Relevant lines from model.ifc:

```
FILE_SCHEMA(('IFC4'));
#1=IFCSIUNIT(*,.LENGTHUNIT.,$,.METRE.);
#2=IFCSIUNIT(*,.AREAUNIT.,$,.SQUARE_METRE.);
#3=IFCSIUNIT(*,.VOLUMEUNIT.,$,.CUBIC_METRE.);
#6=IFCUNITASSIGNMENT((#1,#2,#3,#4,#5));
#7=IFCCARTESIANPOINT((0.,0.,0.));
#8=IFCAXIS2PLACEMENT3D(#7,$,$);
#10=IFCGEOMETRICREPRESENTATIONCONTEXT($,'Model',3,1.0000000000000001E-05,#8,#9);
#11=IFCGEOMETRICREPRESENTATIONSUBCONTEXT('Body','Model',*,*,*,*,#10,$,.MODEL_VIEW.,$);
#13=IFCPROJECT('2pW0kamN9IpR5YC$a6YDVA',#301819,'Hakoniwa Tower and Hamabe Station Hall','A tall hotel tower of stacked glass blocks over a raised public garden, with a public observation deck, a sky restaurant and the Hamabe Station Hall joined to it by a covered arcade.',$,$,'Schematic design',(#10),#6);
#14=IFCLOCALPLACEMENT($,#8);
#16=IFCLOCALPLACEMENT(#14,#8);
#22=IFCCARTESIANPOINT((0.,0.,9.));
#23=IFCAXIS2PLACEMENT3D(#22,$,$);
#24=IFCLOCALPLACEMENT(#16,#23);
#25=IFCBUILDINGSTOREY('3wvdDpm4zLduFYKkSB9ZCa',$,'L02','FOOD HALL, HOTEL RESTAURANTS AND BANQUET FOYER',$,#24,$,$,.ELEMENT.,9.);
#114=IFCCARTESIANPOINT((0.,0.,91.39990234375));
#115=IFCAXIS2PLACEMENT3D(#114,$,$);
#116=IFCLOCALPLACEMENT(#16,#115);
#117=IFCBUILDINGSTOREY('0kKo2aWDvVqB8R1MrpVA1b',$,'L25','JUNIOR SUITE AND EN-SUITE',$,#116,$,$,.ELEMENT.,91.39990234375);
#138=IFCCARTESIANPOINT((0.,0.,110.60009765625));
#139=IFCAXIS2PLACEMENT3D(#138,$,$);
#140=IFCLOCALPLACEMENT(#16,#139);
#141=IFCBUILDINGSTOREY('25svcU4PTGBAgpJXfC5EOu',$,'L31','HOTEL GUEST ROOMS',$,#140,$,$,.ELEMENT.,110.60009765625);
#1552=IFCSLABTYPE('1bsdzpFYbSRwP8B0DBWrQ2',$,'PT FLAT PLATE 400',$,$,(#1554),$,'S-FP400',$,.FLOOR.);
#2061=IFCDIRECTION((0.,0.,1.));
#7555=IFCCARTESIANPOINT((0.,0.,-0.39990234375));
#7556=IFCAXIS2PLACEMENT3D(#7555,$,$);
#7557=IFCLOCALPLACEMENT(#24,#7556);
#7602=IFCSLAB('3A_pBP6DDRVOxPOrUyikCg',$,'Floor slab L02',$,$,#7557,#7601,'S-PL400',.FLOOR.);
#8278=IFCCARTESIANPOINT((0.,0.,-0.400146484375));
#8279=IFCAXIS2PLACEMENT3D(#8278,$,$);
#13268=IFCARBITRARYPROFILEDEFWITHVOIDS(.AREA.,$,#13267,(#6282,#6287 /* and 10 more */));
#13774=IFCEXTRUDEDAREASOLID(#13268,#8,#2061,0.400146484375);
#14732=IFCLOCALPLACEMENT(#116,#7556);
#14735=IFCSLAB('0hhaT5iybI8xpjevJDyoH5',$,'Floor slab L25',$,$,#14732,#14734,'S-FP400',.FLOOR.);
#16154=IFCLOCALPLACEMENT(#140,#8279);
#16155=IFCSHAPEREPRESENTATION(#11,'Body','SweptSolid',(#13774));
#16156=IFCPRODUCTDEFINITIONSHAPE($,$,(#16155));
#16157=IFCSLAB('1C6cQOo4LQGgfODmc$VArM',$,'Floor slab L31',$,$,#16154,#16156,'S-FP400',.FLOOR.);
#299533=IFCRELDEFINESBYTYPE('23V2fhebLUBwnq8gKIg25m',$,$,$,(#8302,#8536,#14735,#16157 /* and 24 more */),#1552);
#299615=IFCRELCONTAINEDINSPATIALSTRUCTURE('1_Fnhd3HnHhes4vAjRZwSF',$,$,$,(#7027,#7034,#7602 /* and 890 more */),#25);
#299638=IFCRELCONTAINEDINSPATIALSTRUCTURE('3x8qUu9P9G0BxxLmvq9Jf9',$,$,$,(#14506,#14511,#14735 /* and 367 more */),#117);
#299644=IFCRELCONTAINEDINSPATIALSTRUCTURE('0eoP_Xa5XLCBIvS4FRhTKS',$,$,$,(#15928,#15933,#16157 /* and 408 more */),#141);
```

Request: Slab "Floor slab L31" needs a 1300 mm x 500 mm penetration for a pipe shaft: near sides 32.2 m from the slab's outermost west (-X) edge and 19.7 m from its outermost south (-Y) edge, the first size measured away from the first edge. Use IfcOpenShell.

```python
import numpy as np
import ifcopenshell
import ifcopenshell.api.feature
import ifcopenshell.api.geometry
import ifcopenshell.api.root
import ifcopenshell.geom
import ifcopenshell.util.placement
import ifcopenshell.util.representation
import ifcopenshell.util.shape
import ifcopenshell.util.unit

model = ifcopenshell.open("model.ifc")
unit_scale = ifcopenshell.util.unit.calculate_unit_scale(model)
settings = ifcopenshell.geom.settings()


def volume(element):
    """Net volume in cubic metres, openings subtracted."""
    shape = ifcopenshell.geom.create_shape(settings, element)
    return ifcopenshell.util.shape.get_volume(shape.geometry)


slab = model.by_guid("1C6cQOo4LQGgfODmc$VArM")
before = volume(slab)

# Extent in the slab's own axes, in metres. The edges named are its -X and -Y sides.
slab_shape = ifcopenshell.geom.create_shape(settings, slab)
vertices = ifcopenshell.util.shape.get_vertices(slab_shape.geometry)
x_min, y_min, bottom = vertices.min(axis=0)
top = vertices[:, 2].max()

opening = ifcopenshell.api.root.create_entity(model, ifc_class="IfcOpeningElement", name="Pipe shaft opening", predefined_type="OPENING")
context = ifcopenshell.util.representation.get_context(model, "Model", "Body", "MODEL_VIEW")
width, depth = 1.3, 0.5
outline = [(0.0, 0.0), (width, 0.0), (width, depth), (0.0, depth), (0.0, 0.0)]
# Overshoot both faces by 50 mm so the cut is clean.
shape = ifcopenshell.api.geometry.add_slab_representation(
    model, context=context, depth=top - bottom + 0.1, polyline=outline
)
ifcopenshell.api.geometry.assign_representation(model, product=opening, representation=shape)

matrix = ifcopenshell.util.placement.get_local_placement(slab.ObjectPlacement)
matrix[:, 3] = matrix @ np.append(np.array([x_min + 32.2, y_min + 19.7, bottom - 0.05]) / unit_scale, 1.0)
ifcopenshell.api.geometry.edit_object_placement(model, product=opening, matrix=matrix, is_si=False)
ifcopenshell.api.feature.add_feature(model, feature=opening, element=slab)

after = volume(slab)

print(f"slab volume {before:.3f} -> {after:.3f} m3")

model.write("model_v2.ifc")
```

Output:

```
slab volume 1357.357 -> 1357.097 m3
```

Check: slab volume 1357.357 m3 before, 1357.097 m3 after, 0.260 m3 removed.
